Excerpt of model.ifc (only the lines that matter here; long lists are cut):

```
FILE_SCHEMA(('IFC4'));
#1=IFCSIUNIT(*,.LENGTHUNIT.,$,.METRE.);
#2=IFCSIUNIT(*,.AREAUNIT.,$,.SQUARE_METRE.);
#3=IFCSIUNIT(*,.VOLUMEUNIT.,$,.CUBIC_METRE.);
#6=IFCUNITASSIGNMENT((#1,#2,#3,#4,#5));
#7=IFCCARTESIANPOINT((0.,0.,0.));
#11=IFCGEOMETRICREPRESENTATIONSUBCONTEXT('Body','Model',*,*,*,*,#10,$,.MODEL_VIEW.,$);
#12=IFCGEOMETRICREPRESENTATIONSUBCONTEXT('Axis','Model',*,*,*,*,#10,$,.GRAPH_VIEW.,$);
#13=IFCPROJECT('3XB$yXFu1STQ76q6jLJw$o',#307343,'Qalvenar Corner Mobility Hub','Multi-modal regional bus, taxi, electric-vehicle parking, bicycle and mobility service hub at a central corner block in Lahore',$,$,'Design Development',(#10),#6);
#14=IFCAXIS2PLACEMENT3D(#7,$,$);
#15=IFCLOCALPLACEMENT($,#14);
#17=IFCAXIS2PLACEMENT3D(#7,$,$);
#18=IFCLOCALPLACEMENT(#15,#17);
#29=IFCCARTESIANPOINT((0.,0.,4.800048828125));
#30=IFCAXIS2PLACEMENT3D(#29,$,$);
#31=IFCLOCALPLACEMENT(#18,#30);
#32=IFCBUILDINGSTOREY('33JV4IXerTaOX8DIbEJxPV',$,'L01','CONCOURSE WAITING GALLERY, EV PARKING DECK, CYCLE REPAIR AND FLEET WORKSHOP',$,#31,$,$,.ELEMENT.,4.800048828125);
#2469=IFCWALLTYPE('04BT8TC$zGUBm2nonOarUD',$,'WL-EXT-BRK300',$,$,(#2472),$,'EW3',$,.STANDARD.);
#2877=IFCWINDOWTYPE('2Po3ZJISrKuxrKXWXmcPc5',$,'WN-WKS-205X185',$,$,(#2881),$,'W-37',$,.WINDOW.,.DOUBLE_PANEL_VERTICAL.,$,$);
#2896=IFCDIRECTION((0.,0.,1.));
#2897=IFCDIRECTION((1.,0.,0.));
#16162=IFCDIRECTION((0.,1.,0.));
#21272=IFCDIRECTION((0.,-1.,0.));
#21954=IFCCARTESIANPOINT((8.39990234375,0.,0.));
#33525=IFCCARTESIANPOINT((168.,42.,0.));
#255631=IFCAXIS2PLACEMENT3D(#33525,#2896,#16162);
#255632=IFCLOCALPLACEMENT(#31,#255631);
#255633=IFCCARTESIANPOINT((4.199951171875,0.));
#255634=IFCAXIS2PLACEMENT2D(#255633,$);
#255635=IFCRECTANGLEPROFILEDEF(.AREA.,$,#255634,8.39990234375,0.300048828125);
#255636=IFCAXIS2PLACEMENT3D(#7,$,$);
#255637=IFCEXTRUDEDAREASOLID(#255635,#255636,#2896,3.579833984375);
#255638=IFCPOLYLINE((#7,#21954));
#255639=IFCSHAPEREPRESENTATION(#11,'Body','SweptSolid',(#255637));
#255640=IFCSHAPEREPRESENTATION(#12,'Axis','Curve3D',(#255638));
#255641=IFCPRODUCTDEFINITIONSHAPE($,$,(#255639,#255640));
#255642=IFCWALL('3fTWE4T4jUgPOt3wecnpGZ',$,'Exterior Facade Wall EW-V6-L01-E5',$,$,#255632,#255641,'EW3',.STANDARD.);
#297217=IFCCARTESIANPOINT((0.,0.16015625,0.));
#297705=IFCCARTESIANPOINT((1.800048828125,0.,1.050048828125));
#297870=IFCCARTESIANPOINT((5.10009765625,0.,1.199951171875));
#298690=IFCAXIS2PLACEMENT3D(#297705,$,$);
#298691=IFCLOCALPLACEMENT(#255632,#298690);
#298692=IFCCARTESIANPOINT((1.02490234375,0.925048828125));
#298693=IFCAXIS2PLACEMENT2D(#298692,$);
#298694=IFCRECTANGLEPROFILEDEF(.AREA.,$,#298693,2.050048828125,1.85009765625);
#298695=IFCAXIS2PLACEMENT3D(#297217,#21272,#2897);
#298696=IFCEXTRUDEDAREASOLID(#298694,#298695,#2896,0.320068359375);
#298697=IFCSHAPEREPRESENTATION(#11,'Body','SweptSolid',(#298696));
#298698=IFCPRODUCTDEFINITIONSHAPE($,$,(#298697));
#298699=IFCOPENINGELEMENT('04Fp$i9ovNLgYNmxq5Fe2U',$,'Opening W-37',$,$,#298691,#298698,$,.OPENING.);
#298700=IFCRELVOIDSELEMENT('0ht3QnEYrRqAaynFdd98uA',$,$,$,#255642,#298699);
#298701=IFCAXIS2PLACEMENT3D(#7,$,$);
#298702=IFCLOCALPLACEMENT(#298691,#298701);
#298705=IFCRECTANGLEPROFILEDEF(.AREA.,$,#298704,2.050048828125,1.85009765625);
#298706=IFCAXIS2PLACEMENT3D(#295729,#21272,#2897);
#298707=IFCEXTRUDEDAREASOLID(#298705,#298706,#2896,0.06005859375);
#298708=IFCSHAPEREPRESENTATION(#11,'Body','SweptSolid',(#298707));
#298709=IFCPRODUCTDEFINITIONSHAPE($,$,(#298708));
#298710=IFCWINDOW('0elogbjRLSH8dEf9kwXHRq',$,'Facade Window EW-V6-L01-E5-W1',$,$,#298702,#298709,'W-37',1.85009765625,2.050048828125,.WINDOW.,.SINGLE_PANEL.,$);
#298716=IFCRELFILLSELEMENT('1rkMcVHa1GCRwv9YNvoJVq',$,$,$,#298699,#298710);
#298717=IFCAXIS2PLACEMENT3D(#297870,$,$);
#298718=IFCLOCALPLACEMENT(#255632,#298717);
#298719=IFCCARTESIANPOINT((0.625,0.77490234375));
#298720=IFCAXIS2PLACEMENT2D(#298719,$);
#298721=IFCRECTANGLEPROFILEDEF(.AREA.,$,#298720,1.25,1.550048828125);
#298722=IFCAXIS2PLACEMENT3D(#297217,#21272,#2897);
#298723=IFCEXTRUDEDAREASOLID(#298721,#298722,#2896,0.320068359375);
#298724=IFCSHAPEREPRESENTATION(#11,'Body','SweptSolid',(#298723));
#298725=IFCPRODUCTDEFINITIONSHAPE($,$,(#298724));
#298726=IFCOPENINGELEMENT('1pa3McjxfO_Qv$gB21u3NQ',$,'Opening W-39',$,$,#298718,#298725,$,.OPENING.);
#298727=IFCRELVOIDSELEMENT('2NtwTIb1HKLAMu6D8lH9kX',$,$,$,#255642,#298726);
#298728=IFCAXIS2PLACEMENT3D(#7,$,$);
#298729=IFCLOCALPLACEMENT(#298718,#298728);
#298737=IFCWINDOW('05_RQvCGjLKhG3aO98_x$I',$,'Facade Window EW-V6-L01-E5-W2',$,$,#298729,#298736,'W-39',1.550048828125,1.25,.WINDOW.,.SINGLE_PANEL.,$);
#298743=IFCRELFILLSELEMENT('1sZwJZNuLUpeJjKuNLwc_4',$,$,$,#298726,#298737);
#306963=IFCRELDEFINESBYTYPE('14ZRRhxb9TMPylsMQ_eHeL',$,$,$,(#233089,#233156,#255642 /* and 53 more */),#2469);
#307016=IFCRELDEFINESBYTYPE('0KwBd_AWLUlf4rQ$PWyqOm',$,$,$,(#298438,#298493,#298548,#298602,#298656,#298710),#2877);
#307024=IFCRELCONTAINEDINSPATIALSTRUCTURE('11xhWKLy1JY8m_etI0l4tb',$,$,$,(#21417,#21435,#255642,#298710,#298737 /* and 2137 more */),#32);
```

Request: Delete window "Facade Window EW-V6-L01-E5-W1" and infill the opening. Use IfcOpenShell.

```python
import ifcopenshell
import ifcopenshell.api.feature
import ifcopenshell.api.root
import ifcopenshell.geom
import ifcopenshell.util.shape

model = ifcopenshell.open("model.ifc")
settings = ifcopenshell.geom.settings()


def volume(element):
    """Net volume in cubic metres, openings subtracted."""
    shape = ifcopenshell.geom.create_shape(settings, element)
    return ifcopenshell.util.shape.get_volume(shape.geometry)


window = model.by_guid("0elogbjRLSH8dEf9kwXHRq")
opening = window.FillsVoids[0].RelatingOpeningElement
wall = opening.VoidsElements[0].RelatingBuildingElement
before = volume(wall)

ifcopenshell.api.root.remove_product(model, product=window)
ifcopenshell.api.feature.remove_feature(model, feature=opening)

after = volume(wall)

print(f"wall volume {before:.3f} -> {after:.3f} m3")

model.write("model_updated.ifc")
```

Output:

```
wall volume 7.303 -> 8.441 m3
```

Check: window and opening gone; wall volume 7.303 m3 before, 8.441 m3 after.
